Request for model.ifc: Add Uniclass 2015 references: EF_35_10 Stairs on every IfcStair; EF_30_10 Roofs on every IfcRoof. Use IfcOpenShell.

First a look at what the model holds.

```python
import ifcopenshell

model = ifcopenshell.open("model.ifc")
print(model.schema)
print("classifications:", [c.Name for c in model.by_type("IfcClassification")])
for ifc_class in ("IfcDoor", "IfcRoof", "IfcStair", "IfcWall", "IfcWindow"):
    print(ifc_class, len(model.by_type(ifc_class)))
```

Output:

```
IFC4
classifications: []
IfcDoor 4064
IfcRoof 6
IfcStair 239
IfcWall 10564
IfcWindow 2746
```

```python
import ifcopenshell
import ifcopenshell.api.classification

model = ifcopenshell.open("model.ifc")

system = ifcopenshell.api.classification.add_classification(model, classification="Uniclass 2015")

codes = {
    "IfcStair": ("EF_35_10", "Stairs"),
    "IfcRoof": ("EF_30_10", "Roofs"),
}
for ifc_class, (code, name) in codes.items():
    products = model.by_type(ifc_class)
    ifcopenshell.api.classification.add_reference(
        model, products=products, classification=system, identification=code, name=name
    )
    print(code, len(products))

model.write("model_edited.ifc")
```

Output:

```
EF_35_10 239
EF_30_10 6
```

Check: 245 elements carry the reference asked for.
